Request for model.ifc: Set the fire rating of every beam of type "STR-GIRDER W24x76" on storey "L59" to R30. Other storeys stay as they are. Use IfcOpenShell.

First a look at what the model holds.

```python
import ifcopenshell
import ifcopenshell.util.element

model = ifcopenshell.open("model.ifc")
print(model.schema)
storey = next(s for s in model.by_type("IfcBuildingStorey") if s.Name == "L59")
beams = [e for e in ifcopenshell.util.element.get_decomposition(storey) if e.is_a("IfcBeam")]
seen = {}
for e in beams:
    element_type = ifcopenshell.util.element.get_type(e)
    key = (element_type.Name if element_type != e and element_type else None, ifcopenshell.util.element.get_pset(e, "Pset_BeamCommon", "FireRating"))
    seen[key] = seen.get(key, 0) + 1
for (name, value), count in sorted(seen.items(), key=str):
    print(count, "x", name, "|", value)
```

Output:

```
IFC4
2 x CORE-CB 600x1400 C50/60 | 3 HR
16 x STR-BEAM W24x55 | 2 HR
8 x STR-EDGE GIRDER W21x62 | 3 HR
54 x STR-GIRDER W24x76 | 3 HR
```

```python
import ifcopenshell
import ifcopenshell.api.pset
import ifcopenshell.util.element

model = ifcopenshell.open("model.ifc")

storey = next(s for s in model.by_type("IfcBuildingStorey") if s.Name == "L59")
beams = [e for e in ifcopenshell.util.element.get_decomposition(storey) if e.is_a("IfcBeam")]

count = 0
for e in beams:
    element_type = ifcopenshell.util.element.get_type(e)
    if element_type in (None, e) or element_type.Name != "STR-GIRDER W24x76":
        continue
    found = ifcopenshell.util.element.get_pset(e, "Pset_BeamCommon", should_inherit=False)
    if found:
        pset = model.by_id(found["id"])
        if len(ifcopenshell.util.element.get_elements_by_pset(pset)) > 1:
            pset = ifcopenshell.api.pset.unshare_pset(model, products=[e], pset=pset)[0]
    else:
        pset = ifcopenshell.api.pset.add_pset(model, product=e, name="Pset_BeamCommon")
    ifcopenshell.api.pset.edit_pset(model, pset=pset, properties={"FireRating": "R30"})
    count += 1

print(count, "beams updated")

model.write("model-out.ifc")
```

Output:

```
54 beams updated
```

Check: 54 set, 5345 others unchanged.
